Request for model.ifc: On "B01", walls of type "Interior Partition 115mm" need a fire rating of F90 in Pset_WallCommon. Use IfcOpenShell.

First a look at what the model holds.

```python
import ifcopenshell
import ifcopenshell.util.element

model = ifcopenshell.open("model.ifc")
print(model.schema)
storey = next(s for s in model.by_type("IfcBuildingStorey") if s.Name == "B01")
walls = [e for e in ifcopenshell.util.element.get_decomposition(storey) if e.is_a("IfcWall")]
seen = {}
for e in walls:
    element_type = ifcopenshell.util.element.get_type(e)
    key = (element_type.Name if element_type != e and element_type else None, ifcopenshell.util.element.get_pset(e, "Pset_WallCommon", "FireRating"))
    seen[key] = seen.get(key, 0) + 1
for (name, value), count in sorted(seen.items(), key=str):
    print(count, "x", name, "|", value)
```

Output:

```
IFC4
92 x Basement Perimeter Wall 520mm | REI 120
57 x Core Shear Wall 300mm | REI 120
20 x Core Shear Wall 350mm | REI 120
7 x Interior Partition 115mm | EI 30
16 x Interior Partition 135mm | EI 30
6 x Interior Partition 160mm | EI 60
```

```python
import ifcopenshell
import ifcopenshell.api.pset
import ifcopenshell.util.element

model = ifcopenshell.open("model.ifc")

storey = next(s for s in model.by_type("IfcBuildingStorey") if s.Name == "B01")
walls = [e for e in ifcopenshell.util.element.get_decomposition(storey) if e.is_a("IfcWall")]

count = 0
for e in walls:
    element_type = ifcopenshell.util.element.get_type(e)
    if element_type in (None, e) or element_type.Name != "Interior Partition 115mm":
        continue
    # add_pset returns the element's existing set when there is one.
    pset = ifcopenshell.api.pset.add_pset(model, product=e, name="Pset_WallCommon")
    ifcopenshell.api.pset.edit_pset(model, pset=pset, properties={"FireRating": "F90"})
    count += 1

print(count, "walls updated")

model.write("model-out.ifc")
```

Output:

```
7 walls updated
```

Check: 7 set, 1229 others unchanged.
